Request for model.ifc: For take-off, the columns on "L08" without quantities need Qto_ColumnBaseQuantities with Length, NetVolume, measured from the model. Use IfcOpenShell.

First a look at what the model holds.

```python
import ifcopenshell
import ifcopenshell.util.element
import ifcopenshell.util.unit

model = ifcopenshell.open("model.ifc")
print(model.schema)
for unit_type in ("LENGTHUNIT", "AREAUNIT", "VOLUMEUNIT"):
    print(unit_type, ifcopenshell.util.unit.calculate_unit_scale(model, unit_type))
storey = next(s for s in model.by_type("IfcBuildingStorey") if s.Name == "L08")
columns = [e for e in ifcopenshell.util.element.get_decomposition(storey) if e.is_a("IfcColumn")]
for e in sorted(columns, key=lambda e: e.id()):
    print(e.id(), e.is_a(), e.Name, list(ifcopenshell.util.element.get_psets(e, qtos_only=True)), sep=" | ")
```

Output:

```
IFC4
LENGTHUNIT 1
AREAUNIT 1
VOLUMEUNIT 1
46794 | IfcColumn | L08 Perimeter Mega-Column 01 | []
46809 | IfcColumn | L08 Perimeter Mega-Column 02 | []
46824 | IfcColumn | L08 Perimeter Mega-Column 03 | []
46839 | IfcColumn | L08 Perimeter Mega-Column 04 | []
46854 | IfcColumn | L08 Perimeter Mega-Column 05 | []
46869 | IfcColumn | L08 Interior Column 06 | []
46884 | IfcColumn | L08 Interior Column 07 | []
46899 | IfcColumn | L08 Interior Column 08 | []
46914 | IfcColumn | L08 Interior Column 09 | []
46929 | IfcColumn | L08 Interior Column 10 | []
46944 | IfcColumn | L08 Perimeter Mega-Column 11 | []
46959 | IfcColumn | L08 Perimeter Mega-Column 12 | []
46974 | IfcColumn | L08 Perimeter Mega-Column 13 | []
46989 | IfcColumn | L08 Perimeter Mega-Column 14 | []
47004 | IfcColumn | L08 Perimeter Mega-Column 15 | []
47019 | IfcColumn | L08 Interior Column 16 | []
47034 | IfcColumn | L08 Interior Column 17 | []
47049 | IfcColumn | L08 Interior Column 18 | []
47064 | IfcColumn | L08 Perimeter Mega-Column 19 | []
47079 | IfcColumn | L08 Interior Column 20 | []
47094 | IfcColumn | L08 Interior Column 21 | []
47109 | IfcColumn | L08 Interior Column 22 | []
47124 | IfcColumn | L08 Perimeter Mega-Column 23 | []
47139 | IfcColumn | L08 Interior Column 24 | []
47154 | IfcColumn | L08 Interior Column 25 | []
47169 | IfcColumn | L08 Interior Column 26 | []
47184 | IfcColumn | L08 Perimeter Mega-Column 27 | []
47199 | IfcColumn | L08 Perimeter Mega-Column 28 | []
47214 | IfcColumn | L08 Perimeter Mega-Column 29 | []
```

```python
import ifcopenshell
import ifcopenshell.api.pset
import ifcopenshell.geom
import ifcopenshell.util.element
import ifcopenshell.util.shape
import ifcopenshell.util.unit

model = ifcopenshell.open("model.ifc")
unit_scale = ifcopenshell.util.unit.calculate_unit_scale(model)
volume_scale = ifcopenshell.util.unit.calculate_unit_scale(model, "VOLUMEUNIT")
settings = ifcopenshell.geom.settings()

storey = next(s for s in model.by_type("IfcBuildingStorey") if s.Name == "L08")
columns = [e for e in ifcopenshell.util.element.get_decomposition(storey) if e.is_a("IfcColumn")]

for e in sorted(columns, key=lambda e: e.id()):
    if ifcopenshell.util.element.get_psets(e, qtos_only=True, should_inherit=False):
        continue
    # Geometry comes back in metres, in the element's own axes.
    shape = ifcopenshell.geom.create_shape(settings, e)
    values = {
        "Length": ifcopenshell.util.shape.get_z(shape.geometry) / unit_scale,
        "NetVolume": ifcopenshell.util.shape.get_volume(shape.geometry) / volume_scale,
    }
    qto = ifcopenshell.api.pset.add_qto(model, product=e, name="Qto_ColumnBaseQuantities")
    ifcopenshell.api.pset.edit_qto(model, qto=qto, properties=values)
    print(e.id(), {k: round(v, 3) for k, v in values.items()})

model.write("model_rev.ifc")
```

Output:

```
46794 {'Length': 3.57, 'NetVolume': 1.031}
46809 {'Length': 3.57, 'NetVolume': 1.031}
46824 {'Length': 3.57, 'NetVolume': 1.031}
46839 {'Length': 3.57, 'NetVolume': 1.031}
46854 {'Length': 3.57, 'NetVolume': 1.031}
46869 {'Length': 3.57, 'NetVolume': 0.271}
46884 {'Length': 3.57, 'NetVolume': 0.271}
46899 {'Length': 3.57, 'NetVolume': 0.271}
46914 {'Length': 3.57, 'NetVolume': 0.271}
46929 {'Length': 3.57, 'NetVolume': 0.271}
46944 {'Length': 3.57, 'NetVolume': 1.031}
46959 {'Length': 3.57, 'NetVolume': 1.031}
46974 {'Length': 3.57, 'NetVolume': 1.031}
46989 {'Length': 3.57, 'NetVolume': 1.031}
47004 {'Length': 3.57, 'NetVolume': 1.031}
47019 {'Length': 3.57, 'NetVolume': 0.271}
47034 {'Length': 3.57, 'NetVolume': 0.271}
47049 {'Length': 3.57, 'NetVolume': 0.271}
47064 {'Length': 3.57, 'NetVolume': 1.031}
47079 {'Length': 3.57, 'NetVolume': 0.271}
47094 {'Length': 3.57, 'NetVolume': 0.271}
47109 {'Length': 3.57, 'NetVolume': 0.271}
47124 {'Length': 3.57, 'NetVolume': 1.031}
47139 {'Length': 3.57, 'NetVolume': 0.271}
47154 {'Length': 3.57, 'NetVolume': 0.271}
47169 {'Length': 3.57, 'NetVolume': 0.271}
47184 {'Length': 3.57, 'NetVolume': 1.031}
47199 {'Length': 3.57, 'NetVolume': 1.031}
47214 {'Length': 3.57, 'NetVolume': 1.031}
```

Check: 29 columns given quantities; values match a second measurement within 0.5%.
